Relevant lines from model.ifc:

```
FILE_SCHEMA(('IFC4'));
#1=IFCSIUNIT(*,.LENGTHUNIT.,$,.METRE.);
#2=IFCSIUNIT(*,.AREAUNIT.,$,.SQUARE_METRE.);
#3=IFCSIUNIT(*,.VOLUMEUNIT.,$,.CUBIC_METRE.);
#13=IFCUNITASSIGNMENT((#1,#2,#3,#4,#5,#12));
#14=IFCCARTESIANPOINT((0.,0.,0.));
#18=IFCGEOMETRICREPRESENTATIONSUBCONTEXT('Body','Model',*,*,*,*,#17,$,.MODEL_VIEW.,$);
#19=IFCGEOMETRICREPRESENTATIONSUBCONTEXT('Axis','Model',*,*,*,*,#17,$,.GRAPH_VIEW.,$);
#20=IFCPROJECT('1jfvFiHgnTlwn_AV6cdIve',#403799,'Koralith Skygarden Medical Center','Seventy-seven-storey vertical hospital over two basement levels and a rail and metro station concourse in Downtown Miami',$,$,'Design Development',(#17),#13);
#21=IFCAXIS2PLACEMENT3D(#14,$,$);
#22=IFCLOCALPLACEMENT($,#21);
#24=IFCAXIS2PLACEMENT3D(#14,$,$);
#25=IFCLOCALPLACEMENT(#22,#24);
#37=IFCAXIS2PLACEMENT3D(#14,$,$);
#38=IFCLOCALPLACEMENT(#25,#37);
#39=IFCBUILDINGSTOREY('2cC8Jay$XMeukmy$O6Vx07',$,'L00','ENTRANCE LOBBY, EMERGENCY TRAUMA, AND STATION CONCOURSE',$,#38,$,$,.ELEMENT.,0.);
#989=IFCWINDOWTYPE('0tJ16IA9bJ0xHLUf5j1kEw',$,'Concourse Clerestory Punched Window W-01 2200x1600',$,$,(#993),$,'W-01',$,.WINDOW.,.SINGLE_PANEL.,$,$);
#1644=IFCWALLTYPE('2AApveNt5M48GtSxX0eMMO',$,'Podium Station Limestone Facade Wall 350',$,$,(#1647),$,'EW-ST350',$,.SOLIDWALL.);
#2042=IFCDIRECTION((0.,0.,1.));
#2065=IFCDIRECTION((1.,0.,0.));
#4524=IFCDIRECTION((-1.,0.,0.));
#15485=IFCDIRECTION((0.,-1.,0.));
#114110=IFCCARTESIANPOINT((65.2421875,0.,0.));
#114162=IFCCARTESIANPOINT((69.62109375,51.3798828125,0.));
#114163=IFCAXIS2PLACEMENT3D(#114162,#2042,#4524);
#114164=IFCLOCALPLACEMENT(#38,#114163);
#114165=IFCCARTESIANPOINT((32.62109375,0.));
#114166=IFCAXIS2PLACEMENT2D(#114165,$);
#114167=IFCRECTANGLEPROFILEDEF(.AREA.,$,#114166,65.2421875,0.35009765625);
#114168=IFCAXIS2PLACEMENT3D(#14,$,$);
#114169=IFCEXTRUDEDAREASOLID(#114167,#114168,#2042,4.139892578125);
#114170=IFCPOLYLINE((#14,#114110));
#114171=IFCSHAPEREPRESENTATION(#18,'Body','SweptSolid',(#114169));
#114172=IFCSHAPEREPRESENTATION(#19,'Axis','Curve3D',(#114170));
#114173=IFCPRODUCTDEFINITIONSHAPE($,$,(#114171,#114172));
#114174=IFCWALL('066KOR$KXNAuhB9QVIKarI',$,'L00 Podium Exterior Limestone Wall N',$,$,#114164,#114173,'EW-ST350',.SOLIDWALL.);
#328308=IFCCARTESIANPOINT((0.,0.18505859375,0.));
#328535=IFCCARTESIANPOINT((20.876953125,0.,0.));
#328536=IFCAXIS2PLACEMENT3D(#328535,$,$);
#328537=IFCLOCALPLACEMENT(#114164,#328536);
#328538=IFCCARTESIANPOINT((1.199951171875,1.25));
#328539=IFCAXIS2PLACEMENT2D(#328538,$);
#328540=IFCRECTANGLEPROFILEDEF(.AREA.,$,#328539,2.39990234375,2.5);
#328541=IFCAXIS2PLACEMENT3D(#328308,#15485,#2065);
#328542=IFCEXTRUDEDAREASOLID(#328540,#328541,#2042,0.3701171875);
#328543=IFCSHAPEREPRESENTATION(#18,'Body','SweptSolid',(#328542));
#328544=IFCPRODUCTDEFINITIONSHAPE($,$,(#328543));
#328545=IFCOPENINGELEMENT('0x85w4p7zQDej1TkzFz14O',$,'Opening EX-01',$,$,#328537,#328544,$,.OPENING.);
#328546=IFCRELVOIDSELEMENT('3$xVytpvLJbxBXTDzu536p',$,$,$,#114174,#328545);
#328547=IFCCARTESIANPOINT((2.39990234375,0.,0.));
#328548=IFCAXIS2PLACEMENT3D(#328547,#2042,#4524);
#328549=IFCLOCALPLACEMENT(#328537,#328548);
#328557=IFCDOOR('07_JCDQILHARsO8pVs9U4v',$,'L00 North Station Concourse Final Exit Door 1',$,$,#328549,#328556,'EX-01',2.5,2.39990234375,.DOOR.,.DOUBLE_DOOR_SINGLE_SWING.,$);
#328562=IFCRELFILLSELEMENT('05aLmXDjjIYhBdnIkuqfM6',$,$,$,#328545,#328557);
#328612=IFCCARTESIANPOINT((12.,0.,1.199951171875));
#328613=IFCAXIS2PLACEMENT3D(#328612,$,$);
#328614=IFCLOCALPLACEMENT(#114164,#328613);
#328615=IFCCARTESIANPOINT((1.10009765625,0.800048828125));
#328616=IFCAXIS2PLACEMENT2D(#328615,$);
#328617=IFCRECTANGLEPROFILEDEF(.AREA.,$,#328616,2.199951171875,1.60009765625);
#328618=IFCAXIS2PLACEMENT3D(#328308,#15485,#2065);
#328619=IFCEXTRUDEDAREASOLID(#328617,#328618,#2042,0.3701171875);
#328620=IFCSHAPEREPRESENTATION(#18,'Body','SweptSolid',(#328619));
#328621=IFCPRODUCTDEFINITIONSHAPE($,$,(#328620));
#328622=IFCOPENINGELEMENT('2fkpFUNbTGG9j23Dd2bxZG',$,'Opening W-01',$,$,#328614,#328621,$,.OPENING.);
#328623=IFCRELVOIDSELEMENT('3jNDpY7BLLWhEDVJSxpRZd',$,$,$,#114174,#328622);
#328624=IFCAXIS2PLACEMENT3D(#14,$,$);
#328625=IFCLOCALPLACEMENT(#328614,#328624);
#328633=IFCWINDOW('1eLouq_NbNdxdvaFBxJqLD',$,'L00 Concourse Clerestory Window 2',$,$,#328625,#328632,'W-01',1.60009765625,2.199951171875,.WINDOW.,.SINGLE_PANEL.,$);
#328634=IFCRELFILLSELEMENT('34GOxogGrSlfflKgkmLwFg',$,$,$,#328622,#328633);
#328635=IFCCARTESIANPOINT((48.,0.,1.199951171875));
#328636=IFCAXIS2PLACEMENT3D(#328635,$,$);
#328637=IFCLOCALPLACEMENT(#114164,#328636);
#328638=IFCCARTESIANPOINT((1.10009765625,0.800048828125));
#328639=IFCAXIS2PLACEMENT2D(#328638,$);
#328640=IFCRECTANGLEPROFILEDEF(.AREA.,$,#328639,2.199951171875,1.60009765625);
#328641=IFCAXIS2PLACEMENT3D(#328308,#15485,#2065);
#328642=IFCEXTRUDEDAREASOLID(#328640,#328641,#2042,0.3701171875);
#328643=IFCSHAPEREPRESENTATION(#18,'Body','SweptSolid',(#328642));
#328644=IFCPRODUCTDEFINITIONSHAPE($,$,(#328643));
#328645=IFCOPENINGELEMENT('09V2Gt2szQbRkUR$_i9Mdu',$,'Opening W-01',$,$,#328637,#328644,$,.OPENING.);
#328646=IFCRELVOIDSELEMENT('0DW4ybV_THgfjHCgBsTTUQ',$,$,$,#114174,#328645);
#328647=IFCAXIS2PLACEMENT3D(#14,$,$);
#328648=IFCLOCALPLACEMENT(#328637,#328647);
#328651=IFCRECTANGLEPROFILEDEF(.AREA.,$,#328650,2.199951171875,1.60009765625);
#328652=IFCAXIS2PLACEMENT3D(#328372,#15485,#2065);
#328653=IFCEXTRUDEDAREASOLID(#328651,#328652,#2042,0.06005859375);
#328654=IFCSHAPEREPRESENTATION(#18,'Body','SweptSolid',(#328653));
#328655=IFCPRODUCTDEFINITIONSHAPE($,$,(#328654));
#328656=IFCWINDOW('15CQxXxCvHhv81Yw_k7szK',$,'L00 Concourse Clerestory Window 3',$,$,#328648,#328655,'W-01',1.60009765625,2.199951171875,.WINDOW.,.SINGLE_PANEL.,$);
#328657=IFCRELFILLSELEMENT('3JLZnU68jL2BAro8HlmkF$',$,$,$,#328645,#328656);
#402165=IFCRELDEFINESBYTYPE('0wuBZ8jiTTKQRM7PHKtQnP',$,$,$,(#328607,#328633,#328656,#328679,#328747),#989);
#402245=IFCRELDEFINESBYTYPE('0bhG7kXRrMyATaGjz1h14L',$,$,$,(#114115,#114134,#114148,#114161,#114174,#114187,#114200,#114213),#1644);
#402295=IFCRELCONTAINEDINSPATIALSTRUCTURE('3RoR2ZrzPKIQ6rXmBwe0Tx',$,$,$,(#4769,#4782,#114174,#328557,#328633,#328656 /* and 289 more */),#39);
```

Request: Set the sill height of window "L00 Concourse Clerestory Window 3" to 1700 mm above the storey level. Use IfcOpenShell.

```python
import numpy as np
import ifcopenshell
import ifcopenshell.api.geometry
import ifcopenshell.geom
import ifcopenshell.util.element
import ifcopenshell.util.placement
import ifcopenshell.util.shape
import ifcopenshell.util.unit

model = ifcopenshell.open("model.ifc")
unit_scale = ifcopenshell.util.unit.calculate_unit_scale(model)

window = model.by_guid("15CQxXxCvHhv81Yw_k7szK")
opening = window.FillsVoids[0].RelatingOpeningElement
storey = ifcopenshell.util.element.get_container(window, ifc_class="IfcBuildingStorey")
level = ifcopenshell.util.placement.get_local_placement(storey.ObjectPlacement)[2, 3]

# The opening's origin need not be at the sill, so measure its lowest point.
shape = ifcopenshell.geom.create_shape(ifcopenshell.geom.settings(), opening)
bottom = ifcopenshell.util.shape.get_shape_bottom_elevation(shape, shape.geometry) / unit_scale
dz = level + 1.7 / unit_scale - bottom

shift = np.array([0.0, 0.0, dz])
# The window is placed relative to its opening, so it follows when the opening moves.
matrix = ifcopenshell.util.placement.get_local_placement(opening.ObjectPlacement)
matrix[:3, 3] += shift
ifcopenshell.api.geometry.edit_object_placement(
    model, product=opening, matrix=matrix, is_si=False, should_transform_children=True
)

print(f"moved by {dz * unit_scale:+.3f} m")

model.write("model_updated.ifc")
```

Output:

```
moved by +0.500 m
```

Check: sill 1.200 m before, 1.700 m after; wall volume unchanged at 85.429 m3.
